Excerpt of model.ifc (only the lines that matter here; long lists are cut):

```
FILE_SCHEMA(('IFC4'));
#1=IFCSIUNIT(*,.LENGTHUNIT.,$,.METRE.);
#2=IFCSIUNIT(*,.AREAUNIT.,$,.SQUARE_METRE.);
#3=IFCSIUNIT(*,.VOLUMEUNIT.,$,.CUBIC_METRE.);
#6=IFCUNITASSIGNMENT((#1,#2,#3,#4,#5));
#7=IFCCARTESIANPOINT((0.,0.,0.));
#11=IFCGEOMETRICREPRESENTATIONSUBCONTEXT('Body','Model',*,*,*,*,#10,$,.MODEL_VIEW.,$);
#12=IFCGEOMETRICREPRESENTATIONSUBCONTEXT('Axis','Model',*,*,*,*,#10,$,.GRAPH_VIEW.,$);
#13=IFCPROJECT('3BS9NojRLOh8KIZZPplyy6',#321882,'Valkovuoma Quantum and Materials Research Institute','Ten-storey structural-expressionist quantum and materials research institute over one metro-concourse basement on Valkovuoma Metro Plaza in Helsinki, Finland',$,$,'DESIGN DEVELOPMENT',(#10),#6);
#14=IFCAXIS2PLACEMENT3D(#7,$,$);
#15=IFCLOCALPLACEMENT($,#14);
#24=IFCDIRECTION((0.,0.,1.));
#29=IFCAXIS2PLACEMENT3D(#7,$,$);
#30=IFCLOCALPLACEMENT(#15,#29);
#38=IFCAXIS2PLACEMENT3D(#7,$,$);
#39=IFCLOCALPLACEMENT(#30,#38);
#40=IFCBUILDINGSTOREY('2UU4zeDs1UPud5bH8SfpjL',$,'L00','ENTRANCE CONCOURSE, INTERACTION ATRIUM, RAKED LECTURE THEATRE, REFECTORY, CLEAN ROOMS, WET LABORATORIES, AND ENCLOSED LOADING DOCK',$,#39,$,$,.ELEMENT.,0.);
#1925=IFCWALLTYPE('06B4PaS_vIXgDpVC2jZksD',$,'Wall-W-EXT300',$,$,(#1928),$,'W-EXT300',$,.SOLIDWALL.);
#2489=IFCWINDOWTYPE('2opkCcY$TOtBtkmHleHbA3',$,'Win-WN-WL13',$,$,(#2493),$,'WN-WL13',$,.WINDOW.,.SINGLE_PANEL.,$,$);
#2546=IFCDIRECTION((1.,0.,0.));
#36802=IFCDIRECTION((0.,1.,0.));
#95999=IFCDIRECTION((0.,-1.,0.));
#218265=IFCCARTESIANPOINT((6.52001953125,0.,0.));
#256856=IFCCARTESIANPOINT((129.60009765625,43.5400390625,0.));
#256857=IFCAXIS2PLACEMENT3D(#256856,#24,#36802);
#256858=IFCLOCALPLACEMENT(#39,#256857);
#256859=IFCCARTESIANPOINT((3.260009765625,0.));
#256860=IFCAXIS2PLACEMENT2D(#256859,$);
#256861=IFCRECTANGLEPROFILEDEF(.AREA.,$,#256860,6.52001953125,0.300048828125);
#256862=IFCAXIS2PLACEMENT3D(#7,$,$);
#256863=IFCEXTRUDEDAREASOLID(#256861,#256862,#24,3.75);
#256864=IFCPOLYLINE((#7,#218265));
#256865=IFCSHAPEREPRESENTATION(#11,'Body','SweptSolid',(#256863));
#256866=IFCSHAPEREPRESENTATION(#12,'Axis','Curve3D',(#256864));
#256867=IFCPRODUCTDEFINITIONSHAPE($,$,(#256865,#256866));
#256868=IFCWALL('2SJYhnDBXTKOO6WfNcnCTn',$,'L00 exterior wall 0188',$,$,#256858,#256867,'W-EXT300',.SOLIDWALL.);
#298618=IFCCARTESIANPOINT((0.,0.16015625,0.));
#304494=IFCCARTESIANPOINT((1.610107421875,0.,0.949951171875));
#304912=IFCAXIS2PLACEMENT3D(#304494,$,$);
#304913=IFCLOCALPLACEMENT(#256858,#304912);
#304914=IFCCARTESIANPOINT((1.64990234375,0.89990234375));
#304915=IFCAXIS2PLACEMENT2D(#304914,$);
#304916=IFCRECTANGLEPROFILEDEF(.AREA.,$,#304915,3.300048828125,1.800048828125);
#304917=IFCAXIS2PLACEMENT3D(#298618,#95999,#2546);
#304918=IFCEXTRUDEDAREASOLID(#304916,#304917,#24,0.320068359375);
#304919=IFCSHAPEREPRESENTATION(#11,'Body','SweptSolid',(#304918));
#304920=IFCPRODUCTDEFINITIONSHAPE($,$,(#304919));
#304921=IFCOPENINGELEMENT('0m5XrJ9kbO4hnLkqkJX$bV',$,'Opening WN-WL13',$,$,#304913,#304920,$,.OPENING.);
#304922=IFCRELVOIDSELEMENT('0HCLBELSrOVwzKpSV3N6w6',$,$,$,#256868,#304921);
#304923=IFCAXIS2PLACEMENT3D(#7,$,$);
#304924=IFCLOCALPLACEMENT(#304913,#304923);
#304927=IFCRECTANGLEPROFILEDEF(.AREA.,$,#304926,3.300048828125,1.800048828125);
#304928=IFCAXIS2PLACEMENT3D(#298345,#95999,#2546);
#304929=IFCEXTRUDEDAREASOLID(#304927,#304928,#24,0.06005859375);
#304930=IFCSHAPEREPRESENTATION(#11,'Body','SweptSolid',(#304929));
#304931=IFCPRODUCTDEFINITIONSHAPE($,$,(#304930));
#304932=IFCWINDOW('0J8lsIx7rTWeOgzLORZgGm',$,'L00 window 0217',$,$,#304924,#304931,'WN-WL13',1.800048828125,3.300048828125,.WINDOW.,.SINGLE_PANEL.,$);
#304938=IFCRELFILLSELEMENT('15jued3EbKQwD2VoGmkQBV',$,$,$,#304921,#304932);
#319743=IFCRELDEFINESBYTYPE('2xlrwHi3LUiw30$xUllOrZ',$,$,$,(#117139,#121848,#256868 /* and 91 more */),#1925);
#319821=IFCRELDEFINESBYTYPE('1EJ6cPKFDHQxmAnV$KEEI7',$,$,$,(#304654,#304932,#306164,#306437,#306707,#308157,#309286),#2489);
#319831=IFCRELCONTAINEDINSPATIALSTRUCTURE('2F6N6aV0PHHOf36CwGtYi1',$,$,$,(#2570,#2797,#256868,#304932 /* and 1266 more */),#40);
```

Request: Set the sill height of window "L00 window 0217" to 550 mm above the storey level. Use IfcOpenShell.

```python
import numpy as np
import ifcopenshell
import ifcopenshell.api.geometry
import ifcopenshell.geom
import ifcopenshell.util.element
import ifcopenshell.util.placement
import ifcopenshell.util.shape
import ifcopenshell.util.unit

model = ifcopenshell.open("model.ifc")
unit_scale = ifcopenshell.util.unit.calculate_unit_scale(model)

window = model.by_guid("0J8lsIx7rTWeOgzLORZgGm")
opening = window.FillsVoids[0].RelatingOpeningElement
storey = ifcopenshell.util.element.get_container(window, ifc_class="IfcBuildingStorey")
level = ifcopenshell.util.placement.get_local_placement(storey.ObjectPlacement)[2, 3]

# The opening's origin need not be at the sill, so measure its lowest point.
shape = ifcopenshell.geom.create_shape(ifcopenshell.geom.settings(), opening)
bottom = ifcopenshell.util.shape.get_shape_bottom_elevation(shape, shape.geometry) / unit_scale
dz = level + 0.55 / unit_scale - bottom

shift = np.array([0.0, 0.0, dz])
# The window is placed relative to its opening, so it follows when the opening moves.
matrix = ifcopenshell.util.placement.get_local_placement(opening.ObjectPlacement)
matrix[:3, 3] += shift
ifcopenshell.api.geometry.edit_object_placement(
    model, product=opening, matrix=matrix, is_si=False, should_transform_children=True
)

print(f"moved by {dz * unit_scale:+.3f} m")

model.write("model_updated.ifc")
```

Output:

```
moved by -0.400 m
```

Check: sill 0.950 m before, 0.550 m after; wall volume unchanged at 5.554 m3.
